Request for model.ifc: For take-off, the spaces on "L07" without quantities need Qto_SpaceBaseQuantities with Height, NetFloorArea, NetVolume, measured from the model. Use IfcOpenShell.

First a look at what the model holds.

```python
import ifcopenshell
import ifcopenshell.util.element
import ifcopenshell.util.unit

model = ifcopenshell.open("model.ifc")
print(model.schema)
for unit_type in ("LENGTHUNIT", "AREAUNIT", "VOLUMEUNIT"):
    print(unit_type, ifcopenshell.util.unit.calculate_unit_scale(model, unit_type))
storey = next(s for s in model.by_type("IfcBuildingStorey") if s.Name == "L07")
spaces = [e for e in ifcopenshell.util.element.get_decomposition(storey) if e.is_a("IfcSpace")]
for e in sorted(spaces, key=lambda e: e.id()):
    print(e.id(), e.is_a(), e.Name, list(ifcopenshell.util.element.get_psets(e, qtos_only=True)), sep=" | ")
```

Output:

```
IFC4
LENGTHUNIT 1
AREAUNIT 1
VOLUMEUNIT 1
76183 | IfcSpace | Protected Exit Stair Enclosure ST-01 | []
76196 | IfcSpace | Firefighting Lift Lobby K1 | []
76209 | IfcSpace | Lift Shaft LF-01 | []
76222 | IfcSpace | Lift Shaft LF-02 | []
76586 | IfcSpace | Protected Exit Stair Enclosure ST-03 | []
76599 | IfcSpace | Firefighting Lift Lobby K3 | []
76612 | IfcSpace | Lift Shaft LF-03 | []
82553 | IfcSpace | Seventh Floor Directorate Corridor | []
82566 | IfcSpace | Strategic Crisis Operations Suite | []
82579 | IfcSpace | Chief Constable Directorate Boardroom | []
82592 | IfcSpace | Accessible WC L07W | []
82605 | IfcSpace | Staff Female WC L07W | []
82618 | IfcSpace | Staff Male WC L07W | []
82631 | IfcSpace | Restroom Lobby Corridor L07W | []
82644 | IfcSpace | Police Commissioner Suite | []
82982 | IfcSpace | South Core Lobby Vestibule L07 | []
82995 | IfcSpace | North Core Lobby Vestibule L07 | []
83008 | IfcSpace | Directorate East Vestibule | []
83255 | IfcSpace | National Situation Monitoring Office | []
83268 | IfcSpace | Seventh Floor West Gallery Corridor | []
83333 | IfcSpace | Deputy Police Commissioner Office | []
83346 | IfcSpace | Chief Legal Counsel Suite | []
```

```python
import ifcopenshell
import ifcopenshell.api.pset
import ifcopenshell.geom
import ifcopenshell.util.element
import ifcopenshell.util.shape
import ifcopenshell.util.unit

model = ifcopenshell.open("model.ifc")
unit_scale = ifcopenshell.util.unit.calculate_unit_scale(model)
area_scale = ifcopenshell.util.unit.calculate_unit_scale(model, "AREAUNIT")
volume_scale = ifcopenshell.util.unit.calculate_unit_scale(model, "VOLUMEUNIT")
settings = ifcopenshell.geom.settings()

storey = next(s for s in model.by_type("IfcBuildingStorey") if s.Name == "L07")
spaces = [e for e in ifcopenshell.util.element.get_decomposition(storey) if e.is_a("IfcSpace")]

for e in sorted(spaces, key=lambda e: e.id()):
    if ifcopenshell.util.element.get_psets(e, qtos_only=True, should_inherit=False):
        continue
    # Geometry comes back in metres, in the element's own axes.
    shape = ifcopenshell.geom.create_shape(settings, e)
    values = {
        "Height": ifcopenshell.util.shape.get_z(shape.geometry) / unit_scale,
        "NetFloorArea": ifcopenshell.util.shape.get_footprint_area(shape.geometry) / area_scale,
        "NetVolume": ifcopenshell.util.shape.get_volume(shape.geometry) / volume_scale,
    }
    qto = ifcopenshell.api.pset.add_qto(model, product=e, name="Qto_SpaceBaseQuantities")
    ifcopenshell.api.pset.edit_qto(model, qto=qto, properties=values)
    print(e.id(), {k: round(v, 3) for k, v in values.items()})

model.write("model_rev.ifc")
```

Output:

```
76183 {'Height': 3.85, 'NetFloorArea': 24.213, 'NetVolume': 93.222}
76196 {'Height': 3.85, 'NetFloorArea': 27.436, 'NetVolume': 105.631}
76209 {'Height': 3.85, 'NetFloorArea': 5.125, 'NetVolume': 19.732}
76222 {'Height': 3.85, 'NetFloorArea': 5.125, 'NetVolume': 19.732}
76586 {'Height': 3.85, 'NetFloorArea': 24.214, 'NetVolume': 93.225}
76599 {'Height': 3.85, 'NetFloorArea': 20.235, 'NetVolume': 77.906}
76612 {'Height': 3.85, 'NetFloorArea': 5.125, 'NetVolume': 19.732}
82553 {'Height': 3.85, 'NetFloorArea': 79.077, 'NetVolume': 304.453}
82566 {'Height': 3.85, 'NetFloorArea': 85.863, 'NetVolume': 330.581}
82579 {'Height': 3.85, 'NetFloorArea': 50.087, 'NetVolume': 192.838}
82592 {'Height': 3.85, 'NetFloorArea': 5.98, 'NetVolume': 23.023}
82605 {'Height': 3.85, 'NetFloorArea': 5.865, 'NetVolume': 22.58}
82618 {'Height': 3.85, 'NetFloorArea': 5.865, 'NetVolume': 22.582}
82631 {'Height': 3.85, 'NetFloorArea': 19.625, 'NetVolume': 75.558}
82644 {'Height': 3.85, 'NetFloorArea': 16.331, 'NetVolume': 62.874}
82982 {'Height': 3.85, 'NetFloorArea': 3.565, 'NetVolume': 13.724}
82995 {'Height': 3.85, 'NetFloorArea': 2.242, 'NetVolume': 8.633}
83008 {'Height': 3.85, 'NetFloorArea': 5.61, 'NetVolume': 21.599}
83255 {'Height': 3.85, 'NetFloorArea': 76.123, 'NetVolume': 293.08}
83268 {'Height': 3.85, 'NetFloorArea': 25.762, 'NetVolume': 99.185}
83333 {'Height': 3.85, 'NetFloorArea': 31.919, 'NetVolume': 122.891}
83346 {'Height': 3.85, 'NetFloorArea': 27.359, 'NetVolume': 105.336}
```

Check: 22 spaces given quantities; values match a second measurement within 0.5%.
